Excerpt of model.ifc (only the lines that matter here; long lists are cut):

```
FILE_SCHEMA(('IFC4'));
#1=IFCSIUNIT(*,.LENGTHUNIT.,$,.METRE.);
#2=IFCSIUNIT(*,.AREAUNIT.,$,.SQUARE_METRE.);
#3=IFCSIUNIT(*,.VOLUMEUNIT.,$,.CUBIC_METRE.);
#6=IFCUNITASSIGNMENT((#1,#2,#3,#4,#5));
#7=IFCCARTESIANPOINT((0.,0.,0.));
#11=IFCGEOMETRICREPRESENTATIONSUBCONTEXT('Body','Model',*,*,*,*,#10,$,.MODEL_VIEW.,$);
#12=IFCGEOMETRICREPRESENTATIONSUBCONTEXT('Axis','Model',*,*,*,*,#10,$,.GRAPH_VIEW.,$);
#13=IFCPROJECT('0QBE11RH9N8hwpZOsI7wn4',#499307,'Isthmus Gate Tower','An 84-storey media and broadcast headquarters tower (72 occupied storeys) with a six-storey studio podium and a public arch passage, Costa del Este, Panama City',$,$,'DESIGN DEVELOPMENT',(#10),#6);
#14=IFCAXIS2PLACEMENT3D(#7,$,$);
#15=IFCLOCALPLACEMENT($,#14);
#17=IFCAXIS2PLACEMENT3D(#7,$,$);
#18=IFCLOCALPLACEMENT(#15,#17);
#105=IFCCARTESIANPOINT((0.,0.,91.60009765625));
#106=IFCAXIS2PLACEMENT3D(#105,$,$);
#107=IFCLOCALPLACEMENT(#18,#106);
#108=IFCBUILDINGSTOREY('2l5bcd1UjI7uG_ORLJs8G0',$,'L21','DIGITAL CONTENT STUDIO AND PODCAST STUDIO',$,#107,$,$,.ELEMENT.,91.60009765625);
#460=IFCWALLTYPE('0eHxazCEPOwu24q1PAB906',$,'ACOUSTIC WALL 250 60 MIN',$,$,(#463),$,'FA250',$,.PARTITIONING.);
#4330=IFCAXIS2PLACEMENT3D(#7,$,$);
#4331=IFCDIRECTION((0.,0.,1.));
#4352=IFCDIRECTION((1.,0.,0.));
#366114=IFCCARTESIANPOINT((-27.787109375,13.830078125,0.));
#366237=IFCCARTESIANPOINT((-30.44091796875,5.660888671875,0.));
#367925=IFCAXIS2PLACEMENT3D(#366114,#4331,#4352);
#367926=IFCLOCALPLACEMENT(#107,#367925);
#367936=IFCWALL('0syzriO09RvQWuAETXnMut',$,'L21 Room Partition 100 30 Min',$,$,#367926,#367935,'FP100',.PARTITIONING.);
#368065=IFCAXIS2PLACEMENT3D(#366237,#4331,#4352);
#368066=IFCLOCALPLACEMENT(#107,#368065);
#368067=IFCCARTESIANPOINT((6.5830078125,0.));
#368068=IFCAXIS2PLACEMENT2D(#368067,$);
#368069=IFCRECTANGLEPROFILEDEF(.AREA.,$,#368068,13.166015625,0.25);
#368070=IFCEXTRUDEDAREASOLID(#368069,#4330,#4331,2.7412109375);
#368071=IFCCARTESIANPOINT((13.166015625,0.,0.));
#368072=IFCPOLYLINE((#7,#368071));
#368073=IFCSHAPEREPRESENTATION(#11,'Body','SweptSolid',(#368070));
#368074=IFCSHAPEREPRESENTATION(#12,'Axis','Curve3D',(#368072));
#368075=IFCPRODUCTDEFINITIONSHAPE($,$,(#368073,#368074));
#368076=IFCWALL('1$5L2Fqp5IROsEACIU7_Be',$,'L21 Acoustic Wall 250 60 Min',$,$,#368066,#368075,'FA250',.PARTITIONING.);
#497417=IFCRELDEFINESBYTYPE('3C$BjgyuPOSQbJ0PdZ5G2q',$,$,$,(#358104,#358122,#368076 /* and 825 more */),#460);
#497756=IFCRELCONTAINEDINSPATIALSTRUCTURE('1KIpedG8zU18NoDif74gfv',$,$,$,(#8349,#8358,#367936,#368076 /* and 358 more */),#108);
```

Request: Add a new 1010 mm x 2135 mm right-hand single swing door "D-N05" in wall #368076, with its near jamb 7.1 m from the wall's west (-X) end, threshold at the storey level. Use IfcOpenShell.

```python
import numpy as np
import ifcopenshell
import ifcopenshell.api.feature
import ifcopenshell.api.geometry
import ifcopenshell.api.root
import ifcopenshell.api.spatial
import ifcopenshell.geom
import ifcopenshell.util.element
import ifcopenshell.util.placement
import ifcopenshell.util.representation
import ifcopenshell.util.shape
import ifcopenshell.util.unit

model = ifcopenshell.open("model.ifc")
unit_scale = ifcopenshell.util.unit.calculate_unit_scale(model)
settings = ifcopenshell.geom.settings()


def volume(element):
    """Net volume in cubic metres, openings subtracted."""
    shape = ifcopenshell.geom.create_shape(settings, element)
    return ifcopenshell.util.shape.get_volume(shape.geometry)


wall = model.by_guid("1$5L2Fqp5IROsEACIU7_Be")
storey = ifcopenshell.util.element.get_container(wall, ifc_class="IfcBuildingStorey")
context = ifcopenshell.util.representation.get_context(model, "Model", "Body", "MODEL_VIEW")
before = volume(wall)

width, height, from_end, sill = 1.01, 2.135, 7.1, 0.0  # metres

# The wall runs along its own X axis, and the end named is its -X end.
wall_shape = ifcopenshell.geom.create_shape(settings, wall)
x, y, z = ifcopenshell.util.shape.get_vertices(wall_shape.geometry).T
start = x.min() + from_end
face, thickness = float(y.min()), float(y.max() - y.min())
wall_matrix = ifcopenshell.util.placement.get_local_placement(wall.ObjectPlacement)
level = ifcopenshell.util.placement.get_local_placement(storey.ObjectPlacement)[2, 3]


def in_wall(x, y):
    """Placement at x, y metres in the wall's axes, at sill height."""
    matrix = wall_matrix.copy()
    matrix[:, 3] = wall_matrix @ np.array([x / unit_scale, y / unit_scale, 0.0, 1.0])
    matrix[2, 3] = level + sill / unit_scale
    return matrix


# Opening: a box that overshoots both wall faces by 50 mm.
opening = ifcopenshell.api.root.create_entity(model, ifc_class="IfcOpeningElement", predefined_type="OPENING")
box = ifcopenshell.api.geometry.add_wall_representation(
    model, context=context, length=width, height=height, thickness=thickness + 0.1
)
ifcopenshell.api.geometry.assign_representation(model, product=opening, representation=box)
ifcopenshell.api.geometry.edit_object_placement(model, product=opening, matrix=in_wall(start, face - 0.05), is_si=False)
ifcopenshell.api.feature.add_feature(model, feature=opening, element=wall)

door = ifcopenshell.api.root.create_entity(model, ifc_class="IfcDoor", name="D-N05", predefined_type="DOOR")
door.OverallWidth, door.OverallHeight = width / unit_scale, height / unit_scale
door.OperationType = "SINGLE_SWING_RIGHT"
body = ifcopenshell.api.geometry.add_door_representation(
    model,
    context=context,
    overall_width=door.OverallWidth,
    overall_height=door.OverallHeight,
    operation_type="SINGLE_SWING_RIGHT",
    lining_properties={"LiningDepth": thickness / unit_scale, "ThresholdDepth": thickness / unit_scale},
)
ifcopenshell.api.geometry.assign_representation(model, product=door, representation=body)
ifcopenshell.api.spatial.assign_container(model, products=[door], relating_structure=storey)
ifcopenshell.api.feature.add_filling(model, opening=opening, element=door)

# The lining spans the wall, so the door starts at the wall face.
ifcopenshell.api.geometry.edit_object_placement(model, product=door, matrix=in_wall(start, face), is_si=False)

after = volume(wall)

print(f"wall volume {before:.3f} -> {after:.3f} m3")

model.write("model_updated.ifc")
```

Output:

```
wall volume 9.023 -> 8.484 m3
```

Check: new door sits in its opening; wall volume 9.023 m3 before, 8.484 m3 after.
